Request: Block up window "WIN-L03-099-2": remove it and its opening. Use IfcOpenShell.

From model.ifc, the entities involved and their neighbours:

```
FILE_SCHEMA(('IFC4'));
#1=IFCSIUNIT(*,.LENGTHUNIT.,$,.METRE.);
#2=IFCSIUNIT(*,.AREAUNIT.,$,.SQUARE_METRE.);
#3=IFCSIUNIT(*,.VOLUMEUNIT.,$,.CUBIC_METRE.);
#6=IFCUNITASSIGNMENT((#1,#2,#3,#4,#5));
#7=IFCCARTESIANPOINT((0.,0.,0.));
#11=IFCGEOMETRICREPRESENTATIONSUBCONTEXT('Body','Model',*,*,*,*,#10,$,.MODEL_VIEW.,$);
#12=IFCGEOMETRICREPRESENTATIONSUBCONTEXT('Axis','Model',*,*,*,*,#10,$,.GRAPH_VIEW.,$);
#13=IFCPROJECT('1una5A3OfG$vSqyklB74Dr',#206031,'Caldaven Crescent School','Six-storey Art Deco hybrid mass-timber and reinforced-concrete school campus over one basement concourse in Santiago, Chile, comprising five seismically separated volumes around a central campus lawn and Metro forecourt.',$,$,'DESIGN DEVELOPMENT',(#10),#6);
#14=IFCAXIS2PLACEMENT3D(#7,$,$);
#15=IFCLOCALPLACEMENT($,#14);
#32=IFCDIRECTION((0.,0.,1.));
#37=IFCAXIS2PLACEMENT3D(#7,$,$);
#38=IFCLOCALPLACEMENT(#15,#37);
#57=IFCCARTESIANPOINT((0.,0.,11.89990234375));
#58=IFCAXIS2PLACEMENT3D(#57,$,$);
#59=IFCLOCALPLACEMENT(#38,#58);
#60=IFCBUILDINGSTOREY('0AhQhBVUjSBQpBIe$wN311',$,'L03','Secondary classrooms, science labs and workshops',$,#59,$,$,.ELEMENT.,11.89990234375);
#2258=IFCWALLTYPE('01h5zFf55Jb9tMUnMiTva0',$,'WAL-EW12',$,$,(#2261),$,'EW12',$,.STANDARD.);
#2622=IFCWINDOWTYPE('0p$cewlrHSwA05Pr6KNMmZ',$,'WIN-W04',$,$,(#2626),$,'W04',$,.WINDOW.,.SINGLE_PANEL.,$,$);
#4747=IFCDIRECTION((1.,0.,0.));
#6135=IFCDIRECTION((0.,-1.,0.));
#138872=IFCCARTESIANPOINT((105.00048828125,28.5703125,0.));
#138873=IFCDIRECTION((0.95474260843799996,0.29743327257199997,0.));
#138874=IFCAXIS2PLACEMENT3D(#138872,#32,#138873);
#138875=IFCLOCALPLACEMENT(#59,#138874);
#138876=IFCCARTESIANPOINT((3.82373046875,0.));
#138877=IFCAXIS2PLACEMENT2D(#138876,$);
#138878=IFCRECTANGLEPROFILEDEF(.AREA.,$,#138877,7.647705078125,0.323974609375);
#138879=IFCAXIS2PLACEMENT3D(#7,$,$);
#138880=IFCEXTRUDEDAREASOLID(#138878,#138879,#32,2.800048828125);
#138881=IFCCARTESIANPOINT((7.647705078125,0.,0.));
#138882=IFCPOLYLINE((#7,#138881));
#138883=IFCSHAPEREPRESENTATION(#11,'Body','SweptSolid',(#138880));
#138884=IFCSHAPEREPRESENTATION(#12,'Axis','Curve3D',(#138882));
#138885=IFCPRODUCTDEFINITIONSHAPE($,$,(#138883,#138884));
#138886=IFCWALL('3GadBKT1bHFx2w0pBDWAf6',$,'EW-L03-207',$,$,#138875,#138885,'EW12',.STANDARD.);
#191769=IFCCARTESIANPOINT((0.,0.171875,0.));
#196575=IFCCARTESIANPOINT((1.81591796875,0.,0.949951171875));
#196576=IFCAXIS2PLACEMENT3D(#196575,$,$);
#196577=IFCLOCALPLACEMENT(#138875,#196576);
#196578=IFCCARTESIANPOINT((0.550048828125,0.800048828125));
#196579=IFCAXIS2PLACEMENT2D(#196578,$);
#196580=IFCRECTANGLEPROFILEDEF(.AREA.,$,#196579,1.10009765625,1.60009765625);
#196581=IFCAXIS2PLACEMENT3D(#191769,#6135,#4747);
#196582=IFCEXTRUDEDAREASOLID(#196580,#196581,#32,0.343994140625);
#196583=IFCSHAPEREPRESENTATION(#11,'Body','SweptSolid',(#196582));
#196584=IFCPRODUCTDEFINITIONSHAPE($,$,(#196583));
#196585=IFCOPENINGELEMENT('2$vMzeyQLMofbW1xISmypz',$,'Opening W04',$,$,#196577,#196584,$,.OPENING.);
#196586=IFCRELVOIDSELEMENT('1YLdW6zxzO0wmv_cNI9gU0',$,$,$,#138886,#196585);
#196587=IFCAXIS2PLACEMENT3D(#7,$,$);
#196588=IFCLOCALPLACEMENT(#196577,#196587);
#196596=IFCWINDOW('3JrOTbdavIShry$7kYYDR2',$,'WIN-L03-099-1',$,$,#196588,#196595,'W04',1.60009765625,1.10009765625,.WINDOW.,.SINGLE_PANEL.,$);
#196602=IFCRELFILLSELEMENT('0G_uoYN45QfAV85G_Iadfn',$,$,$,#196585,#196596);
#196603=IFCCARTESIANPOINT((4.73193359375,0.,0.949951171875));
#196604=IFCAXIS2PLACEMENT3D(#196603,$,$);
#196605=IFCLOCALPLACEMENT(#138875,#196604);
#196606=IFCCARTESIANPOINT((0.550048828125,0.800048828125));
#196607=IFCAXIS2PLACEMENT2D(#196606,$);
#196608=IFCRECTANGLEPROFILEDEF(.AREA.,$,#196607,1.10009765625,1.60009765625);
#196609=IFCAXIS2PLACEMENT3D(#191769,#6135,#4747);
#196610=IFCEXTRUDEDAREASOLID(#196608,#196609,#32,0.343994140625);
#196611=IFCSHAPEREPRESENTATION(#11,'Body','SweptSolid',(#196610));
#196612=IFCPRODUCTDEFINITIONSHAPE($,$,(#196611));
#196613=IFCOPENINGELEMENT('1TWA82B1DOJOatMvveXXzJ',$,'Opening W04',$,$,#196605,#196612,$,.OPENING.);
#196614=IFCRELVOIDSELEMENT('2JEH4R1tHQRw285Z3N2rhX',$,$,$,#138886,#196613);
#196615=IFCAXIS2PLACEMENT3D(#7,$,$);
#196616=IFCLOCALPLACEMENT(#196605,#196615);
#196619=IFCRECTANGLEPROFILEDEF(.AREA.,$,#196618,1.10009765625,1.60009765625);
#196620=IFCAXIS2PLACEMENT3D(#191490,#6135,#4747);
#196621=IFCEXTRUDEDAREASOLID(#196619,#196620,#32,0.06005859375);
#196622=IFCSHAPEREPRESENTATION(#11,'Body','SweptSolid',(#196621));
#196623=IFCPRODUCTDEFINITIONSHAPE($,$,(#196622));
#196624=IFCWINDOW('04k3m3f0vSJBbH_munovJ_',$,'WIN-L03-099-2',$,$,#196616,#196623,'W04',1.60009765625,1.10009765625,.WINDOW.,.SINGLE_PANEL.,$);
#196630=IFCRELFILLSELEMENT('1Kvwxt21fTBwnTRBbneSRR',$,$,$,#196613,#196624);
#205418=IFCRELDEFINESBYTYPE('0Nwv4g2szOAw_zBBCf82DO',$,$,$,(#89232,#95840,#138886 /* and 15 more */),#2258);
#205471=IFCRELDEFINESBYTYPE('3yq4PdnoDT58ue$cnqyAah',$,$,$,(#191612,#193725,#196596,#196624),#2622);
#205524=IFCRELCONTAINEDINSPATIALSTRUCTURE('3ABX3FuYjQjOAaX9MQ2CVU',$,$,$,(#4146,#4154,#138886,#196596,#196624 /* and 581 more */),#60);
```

```python
import ifcopenshell
import ifcopenshell.api.feature
import ifcopenshell.api.root
import ifcopenshell.geom
import ifcopenshell.util.shape

model = ifcopenshell.open("model.ifc")
settings = ifcopenshell.geom.settings()


def volume(element):
    """Net volume in cubic metres, openings subtracted."""
    shape = ifcopenshell.geom.create_shape(settings, element)
    return ifcopenshell.util.shape.get_volume(shape.geometry)


window = model.by_id(196624)
opening = window.FillsVoids[0].RelatingOpeningElement
wall = opening.VoidsElements[0].RelatingBuildingElement
before = volume(wall)

ifcopenshell.api.root.remove_product(model, product=window)
ifcopenshell.api.feature.remove_feature(model, feature=opening)

after = volume(wall)

print(f"wall volume {before:.3f} -> {after:.3f} m3")

model.write("model_updated.ifc")
```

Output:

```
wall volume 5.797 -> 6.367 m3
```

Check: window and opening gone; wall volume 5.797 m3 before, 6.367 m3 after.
